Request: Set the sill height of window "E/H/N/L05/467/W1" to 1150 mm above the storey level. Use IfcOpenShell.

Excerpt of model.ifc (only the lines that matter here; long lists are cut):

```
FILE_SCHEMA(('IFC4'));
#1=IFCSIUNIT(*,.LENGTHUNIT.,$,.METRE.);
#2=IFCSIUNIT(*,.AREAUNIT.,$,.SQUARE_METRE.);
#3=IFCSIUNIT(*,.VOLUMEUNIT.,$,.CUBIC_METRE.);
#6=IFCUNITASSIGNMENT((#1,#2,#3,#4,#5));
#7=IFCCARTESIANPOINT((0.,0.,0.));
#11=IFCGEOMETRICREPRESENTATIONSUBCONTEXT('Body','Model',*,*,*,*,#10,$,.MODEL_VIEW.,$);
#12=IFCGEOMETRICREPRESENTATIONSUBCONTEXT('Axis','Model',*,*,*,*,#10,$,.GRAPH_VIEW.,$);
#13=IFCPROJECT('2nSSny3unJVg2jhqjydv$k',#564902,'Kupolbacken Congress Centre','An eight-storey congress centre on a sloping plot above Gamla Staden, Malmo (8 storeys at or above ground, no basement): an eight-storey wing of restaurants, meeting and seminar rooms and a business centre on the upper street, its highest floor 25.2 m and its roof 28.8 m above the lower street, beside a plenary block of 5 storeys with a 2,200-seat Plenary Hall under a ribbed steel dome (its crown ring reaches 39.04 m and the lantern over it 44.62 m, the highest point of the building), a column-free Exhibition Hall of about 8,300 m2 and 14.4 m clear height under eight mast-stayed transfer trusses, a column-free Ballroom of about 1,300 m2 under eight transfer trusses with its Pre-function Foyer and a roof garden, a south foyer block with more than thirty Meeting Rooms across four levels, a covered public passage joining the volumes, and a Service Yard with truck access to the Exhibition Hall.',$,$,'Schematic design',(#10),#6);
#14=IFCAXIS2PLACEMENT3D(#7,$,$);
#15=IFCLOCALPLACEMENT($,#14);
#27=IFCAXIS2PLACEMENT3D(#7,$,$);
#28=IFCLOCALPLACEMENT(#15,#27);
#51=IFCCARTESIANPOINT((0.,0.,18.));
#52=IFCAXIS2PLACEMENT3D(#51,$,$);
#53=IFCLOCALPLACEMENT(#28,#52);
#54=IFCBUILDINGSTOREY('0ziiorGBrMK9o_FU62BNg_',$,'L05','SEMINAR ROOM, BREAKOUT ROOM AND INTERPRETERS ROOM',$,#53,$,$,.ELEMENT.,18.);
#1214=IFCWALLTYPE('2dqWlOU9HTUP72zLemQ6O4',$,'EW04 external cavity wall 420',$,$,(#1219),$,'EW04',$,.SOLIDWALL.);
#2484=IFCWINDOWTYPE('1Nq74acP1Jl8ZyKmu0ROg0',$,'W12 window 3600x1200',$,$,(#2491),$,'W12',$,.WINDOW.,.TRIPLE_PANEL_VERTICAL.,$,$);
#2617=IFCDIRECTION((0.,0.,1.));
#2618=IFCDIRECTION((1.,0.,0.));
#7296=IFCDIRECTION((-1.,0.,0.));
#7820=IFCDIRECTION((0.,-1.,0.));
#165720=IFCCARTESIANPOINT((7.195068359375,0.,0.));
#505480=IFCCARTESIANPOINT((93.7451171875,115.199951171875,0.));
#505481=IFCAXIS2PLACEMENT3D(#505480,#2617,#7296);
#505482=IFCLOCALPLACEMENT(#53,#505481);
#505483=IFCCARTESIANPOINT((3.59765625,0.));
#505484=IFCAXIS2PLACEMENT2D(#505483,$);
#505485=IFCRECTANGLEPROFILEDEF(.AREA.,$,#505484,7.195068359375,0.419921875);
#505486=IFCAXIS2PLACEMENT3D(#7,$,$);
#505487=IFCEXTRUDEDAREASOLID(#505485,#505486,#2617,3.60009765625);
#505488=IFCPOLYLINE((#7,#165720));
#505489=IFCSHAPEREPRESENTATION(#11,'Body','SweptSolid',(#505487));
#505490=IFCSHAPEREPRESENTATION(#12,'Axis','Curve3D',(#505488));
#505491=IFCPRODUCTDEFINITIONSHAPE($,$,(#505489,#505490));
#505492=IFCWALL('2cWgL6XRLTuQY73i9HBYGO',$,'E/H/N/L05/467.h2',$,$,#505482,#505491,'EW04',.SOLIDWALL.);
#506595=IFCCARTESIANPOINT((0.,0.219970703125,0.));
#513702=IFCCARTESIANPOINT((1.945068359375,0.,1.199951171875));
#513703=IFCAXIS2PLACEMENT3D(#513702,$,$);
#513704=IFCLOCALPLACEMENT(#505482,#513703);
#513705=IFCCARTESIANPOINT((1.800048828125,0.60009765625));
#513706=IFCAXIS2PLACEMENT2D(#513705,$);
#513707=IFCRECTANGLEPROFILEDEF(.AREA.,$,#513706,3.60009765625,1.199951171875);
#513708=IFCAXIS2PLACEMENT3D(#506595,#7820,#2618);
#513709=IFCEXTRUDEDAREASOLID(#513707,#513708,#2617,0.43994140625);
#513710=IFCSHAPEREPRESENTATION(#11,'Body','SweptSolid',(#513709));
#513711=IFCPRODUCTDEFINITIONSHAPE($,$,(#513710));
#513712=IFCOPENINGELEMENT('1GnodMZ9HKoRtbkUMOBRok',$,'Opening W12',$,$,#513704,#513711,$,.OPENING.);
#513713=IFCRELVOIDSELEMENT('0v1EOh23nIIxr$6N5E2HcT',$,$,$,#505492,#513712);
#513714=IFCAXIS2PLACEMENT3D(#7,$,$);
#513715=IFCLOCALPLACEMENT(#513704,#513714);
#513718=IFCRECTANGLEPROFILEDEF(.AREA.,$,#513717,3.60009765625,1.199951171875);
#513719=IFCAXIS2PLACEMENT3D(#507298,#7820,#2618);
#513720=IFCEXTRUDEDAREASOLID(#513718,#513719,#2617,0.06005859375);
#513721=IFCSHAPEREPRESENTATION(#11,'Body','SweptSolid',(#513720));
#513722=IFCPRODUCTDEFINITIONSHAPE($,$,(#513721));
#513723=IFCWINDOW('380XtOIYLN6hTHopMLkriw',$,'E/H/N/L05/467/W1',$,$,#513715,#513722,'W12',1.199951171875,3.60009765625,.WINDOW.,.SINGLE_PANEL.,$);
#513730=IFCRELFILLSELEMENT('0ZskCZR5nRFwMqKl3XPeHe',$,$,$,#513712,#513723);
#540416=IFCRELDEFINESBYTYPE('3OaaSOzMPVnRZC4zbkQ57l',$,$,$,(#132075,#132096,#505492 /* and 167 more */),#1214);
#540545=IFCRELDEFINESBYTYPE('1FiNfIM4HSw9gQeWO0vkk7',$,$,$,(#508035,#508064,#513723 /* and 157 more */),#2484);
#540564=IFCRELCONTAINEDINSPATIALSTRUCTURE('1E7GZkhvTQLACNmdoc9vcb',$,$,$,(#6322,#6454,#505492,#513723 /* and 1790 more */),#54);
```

```python
import numpy as np
import ifcopenshell
import ifcopenshell.api.geometry
import ifcopenshell.geom
import ifcopenshell.util.element
import ifcopenshell.util.placement
import ifcopenshell.util.shape
import ifcopenshell.util.unit

model = ifcopenshell.open("model.ifc")
unit_scale = ifcopenshell.util.unit.calculate_unit_scale(model)

window = model.by_guid("380XtOIYLN6hTHopMLkriw")
opening = window.FillsVoids[0].RelatingOpeningElement
storey = ifcopenshell.util.element.get_container(window, ifc_class="IfcBuildingStorey")
level = ifcopenshell.util.placement.get_local_placement(storey.ObjectPlacement)[2, 3]

# The opening's origin need not be at the sill, so measure its lowest point.
shape = ifcopenshell.geom.create_shape(ifcopenshell.geom.settings(), opening)
bottom = ifcopenshell.util.shape.get_shape_bottom_elevation(shape, shape.geometry) / unit_scale
dz = level + 1.15 - bottom

shift = np.array([0.0, 0.0, dz])
# The window is placed relative to its opening, so it follows when the opening moves.
matrix = ifcopenshell.util.placement.get_local_placement(opening.ObjectPlacement)
matrix[:3, 3] += shift
ifcopenshell.api.geometry.edit_object_placement(
    model, product=opening, matrix=matrix, is_si=False, should_transform_children=True
)

print(f"moved by {dz * unit_scale:+.3f} m")

model.write("model_v2.ifc")
```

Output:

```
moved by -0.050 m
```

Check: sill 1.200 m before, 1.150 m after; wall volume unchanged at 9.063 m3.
